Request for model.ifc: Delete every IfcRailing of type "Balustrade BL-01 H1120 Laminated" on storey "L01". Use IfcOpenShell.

First a look at what the model holds.

```python
import ifcopenshell
import ifcopenshell.util.element

model = ifcopenshell.open("model.ifc")
print(model.schema)
storey = next(s for s in model.by_type("IfcBuildingStorey") if s.Name == "L01")
railings = [e for e in ifcopenshell.util.element.get_decomposition(storey) if e.is_a("IfcRailing")]
seen = {}
for e in railings:
    element_type = ifcopenshell.util.element.get_type(e)
    name = element_type.Name if element_type not in (None, e) else None
    seen[name] = seen.get(name, 0) + 1
for name, count in sorted(seen.items(), key=str):
    print(count, "x", name)
```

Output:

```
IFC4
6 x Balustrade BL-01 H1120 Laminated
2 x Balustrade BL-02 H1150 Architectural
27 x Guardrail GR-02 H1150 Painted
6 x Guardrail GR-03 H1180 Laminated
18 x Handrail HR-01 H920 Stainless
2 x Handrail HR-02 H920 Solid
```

```python
import ifcopenshell
import ifcopenshell.api.root
import ifcopenshell.util.element

model = ifcopenshell.open("model.ifc")

storey = next(s for s in model.by_type("IfcBuildingStorey") if s.Name == "L01")
railings = [e for e in ifcopenshell.util.element.get_decomposition(storey) if e.is_a("IfcRailing")]
targets = [e for e in railings if (t := ifcopenshell.util.element.get_type(e)) not in (None, e) and t.Name == "Balustrade BL-01 H1120 Laminated"]

for e in targets:
    ifcopenshell.api.root.remove_product(model, product=e)
print(len(targets), "removed")

model.write("model_updated.ifc")
```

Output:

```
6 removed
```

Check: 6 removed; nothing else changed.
